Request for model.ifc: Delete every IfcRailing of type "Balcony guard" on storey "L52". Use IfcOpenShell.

First a look at what the model holds.

```python
import ifcopenshell
import ifcopenshell.util.element

model = ifcopenshell.open("model.ifc")
print(model.schema)
storey = next(s for s in model.by_type("IfcBuildingStorey") if s.Name == "L52")
railings = [e for e in ifcopenshell.util.element.get_decomposition(storey) if e.is_a("IfcRailing")]
seen = {}
for e in railings:
    element_type = ifcopenshell.util.element.get_type(e)
    name = element_type.Name if element_type not in (None, e) else None
    seen[name] = seen.get(name, 0) + 1
for name, count in sorted(seen.items(), key=str):
    print(count, "x", name)
```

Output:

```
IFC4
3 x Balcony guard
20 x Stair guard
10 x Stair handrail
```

```python
import ifcopenshell
import ifcopenshell.api.root
import ifcopenshell.util.element

model = ifcopenshell.open("model.ifc")

storey = next(s for s in model.by_type("IfcBuildingStorey") if s.Name == "L52")
railings = [e for e in ifcopenshell.util.element.get_decomposition(storey) if e.is_a("IfcRailing")]
targets = [e for e in railings if (t := ifcopenshell.util.element.get_type(e)) not in (None, e) and t.Name == "Balcony guard"]

for e in targets:
    ifcopenshell.api.root.remove_product(model, product=e)
print(len(targets), "removed")

model.write("model_v2.ifc")
```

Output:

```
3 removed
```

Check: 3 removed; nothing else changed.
